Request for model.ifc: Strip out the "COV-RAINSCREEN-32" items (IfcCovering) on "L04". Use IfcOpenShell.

First a look at what the model holds.

```python
import ifcopenshell
import ifcopenshell.util.element

model = ifcopenshell.open("model.ifc")
print(model.schema)
storey = next(s for s in model.by_type("IfcBuildingStorey") if s.Name == "L04")
coverings = [e for e in ifcopenshell.util.element.get_decomposition(storey) if e.is_a("IfcCovering")]
seen = {}
for e in coverings:
    element_type = ifcopenshell.util.element.get_type(e)
    name = element_type.Name if element_type not in (None, e) else None
    seen[name] = seen.get(name, 0) + 1
for name, count in sorted(seen.items(), key=str):
    print(count, "x", name)
```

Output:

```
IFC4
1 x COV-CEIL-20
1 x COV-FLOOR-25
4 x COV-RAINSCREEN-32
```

```python
import ifcopenshell
import ifcopenshell.api.root
import ifcopenshell.util.element

model = ifcopenshell.open("model.ifc")

storey = next(s for s in model.by_type("IfcBuildingStorey") if s.Name == "L04")
coverings = [e for e in ifcopenshell.util.element.get_decomposition(storey) if e.is_a("IfcCovering")]
targets = [e for e in coverings if (t := ifcopenshell.util.element.get_type(e)) not in (None, e) and t.Name == "COV-RAINSCREEN-32"]

for e in targets:
    ifcopenshell.api.root.remove_product(model, product=e)
print(len(targets), "removed")

model.write("model_updated.ifc")
```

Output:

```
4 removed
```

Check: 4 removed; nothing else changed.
